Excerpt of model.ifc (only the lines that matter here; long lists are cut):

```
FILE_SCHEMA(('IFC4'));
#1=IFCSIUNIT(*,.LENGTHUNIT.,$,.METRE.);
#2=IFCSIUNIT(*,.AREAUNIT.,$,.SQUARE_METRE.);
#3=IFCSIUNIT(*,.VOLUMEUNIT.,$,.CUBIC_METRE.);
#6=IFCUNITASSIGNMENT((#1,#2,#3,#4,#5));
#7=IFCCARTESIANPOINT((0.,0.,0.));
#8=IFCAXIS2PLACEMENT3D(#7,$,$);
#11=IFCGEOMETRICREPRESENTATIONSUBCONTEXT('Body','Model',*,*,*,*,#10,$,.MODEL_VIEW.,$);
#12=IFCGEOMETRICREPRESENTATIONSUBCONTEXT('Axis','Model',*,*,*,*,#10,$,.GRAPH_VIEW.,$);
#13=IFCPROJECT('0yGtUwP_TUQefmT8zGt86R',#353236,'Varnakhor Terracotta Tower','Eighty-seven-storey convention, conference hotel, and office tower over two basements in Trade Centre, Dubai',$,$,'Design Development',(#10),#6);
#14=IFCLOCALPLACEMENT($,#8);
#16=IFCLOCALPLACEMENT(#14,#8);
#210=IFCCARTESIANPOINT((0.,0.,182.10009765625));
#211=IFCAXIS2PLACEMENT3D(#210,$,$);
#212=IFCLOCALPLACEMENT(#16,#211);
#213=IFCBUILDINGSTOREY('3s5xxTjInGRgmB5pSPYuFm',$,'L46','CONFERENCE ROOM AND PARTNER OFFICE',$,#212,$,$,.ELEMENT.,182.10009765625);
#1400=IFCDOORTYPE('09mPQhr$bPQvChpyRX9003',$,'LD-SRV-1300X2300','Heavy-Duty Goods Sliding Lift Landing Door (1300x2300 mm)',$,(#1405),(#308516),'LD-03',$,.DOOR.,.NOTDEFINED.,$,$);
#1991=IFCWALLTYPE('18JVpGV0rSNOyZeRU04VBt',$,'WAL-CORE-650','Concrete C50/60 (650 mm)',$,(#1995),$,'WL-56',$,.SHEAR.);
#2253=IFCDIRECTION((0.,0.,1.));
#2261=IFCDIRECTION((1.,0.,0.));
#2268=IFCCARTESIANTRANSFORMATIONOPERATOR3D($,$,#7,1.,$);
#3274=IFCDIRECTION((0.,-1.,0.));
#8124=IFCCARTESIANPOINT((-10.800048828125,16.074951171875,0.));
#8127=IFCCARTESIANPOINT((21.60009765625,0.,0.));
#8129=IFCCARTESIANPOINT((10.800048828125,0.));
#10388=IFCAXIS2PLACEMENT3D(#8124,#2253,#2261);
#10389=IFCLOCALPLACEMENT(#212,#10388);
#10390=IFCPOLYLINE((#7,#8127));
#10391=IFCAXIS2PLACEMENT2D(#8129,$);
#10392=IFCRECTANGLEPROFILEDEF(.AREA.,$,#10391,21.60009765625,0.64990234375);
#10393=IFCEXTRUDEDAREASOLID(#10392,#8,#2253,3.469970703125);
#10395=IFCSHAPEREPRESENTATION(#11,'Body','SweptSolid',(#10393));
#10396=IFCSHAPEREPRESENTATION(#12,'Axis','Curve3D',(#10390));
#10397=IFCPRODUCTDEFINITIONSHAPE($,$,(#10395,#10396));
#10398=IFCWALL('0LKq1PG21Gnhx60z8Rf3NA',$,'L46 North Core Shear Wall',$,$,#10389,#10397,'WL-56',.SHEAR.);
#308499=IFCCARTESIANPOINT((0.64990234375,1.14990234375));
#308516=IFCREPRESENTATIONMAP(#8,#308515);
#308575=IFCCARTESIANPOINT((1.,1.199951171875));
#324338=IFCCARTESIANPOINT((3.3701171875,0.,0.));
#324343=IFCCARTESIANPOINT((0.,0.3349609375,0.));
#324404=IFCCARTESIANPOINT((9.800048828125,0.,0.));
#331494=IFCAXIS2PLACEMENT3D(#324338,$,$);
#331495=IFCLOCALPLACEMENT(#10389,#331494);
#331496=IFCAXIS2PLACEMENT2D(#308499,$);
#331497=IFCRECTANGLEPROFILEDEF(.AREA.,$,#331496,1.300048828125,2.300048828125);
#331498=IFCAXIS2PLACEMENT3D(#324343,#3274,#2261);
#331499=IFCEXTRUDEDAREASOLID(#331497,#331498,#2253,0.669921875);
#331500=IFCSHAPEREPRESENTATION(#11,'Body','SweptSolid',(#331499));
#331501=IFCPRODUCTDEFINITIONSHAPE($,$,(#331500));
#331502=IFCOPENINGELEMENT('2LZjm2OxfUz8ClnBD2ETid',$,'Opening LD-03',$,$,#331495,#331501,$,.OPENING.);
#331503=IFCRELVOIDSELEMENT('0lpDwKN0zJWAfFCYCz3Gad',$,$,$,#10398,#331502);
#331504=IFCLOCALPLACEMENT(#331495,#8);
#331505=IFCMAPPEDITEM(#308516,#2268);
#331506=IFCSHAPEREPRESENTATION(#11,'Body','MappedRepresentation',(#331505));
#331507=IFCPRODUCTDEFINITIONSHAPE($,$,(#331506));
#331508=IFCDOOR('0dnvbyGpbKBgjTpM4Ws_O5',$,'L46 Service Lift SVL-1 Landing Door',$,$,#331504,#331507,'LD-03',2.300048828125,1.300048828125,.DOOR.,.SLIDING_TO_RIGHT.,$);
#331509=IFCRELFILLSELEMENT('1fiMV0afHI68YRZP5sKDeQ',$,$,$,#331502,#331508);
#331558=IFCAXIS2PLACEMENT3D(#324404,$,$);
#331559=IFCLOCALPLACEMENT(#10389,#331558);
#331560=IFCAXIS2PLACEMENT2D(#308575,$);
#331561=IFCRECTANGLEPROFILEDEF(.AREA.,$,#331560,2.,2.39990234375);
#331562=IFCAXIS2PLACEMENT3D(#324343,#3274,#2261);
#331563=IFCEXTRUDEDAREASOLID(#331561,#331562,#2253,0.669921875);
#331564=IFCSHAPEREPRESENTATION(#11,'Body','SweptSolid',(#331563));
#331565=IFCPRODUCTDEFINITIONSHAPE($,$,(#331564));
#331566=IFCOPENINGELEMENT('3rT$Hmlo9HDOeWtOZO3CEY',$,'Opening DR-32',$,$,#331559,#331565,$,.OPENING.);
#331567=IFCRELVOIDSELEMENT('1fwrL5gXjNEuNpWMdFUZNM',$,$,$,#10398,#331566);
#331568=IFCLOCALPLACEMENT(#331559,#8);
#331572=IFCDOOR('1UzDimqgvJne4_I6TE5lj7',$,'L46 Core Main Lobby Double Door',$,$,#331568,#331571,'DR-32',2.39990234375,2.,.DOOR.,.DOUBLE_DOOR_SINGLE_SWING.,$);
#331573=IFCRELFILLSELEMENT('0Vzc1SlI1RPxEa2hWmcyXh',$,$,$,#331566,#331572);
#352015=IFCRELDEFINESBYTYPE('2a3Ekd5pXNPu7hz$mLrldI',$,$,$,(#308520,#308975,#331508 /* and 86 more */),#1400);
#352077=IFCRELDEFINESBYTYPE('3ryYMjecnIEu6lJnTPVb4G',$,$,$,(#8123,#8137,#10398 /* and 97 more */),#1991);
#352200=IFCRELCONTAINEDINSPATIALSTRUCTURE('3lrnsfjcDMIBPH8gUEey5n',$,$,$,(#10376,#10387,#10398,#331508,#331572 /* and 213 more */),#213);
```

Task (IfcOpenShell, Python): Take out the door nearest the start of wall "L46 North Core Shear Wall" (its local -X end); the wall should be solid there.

```python
import ifcopenshell
import ifcopenshell.api.feature
import ifcopenshell.api.root
import ifcopenshell.geom
import ifcopenshell.util.shape

model = ifcopenshell.open("model.ifc")
settings = ifcopenshell.geom.settings()


def volume(element):
    """Net volume in cubic metres, openings subtracted."""
    shape = ifcopenshell.geom.create_shape(settings, element)
    return ifcopenshell.util.shape.get_volume(shape.geometry)


door = model.by_guid("0dnvbyGpbKBgjTpM4Ws_O5")
opening = door.FillsVoids[0].RelatingOpeningElement
wall = opening.VoidsElements[0].RelatingBuildingElement
before = volume(wall)

ifcopenshell.api.root.remove_product(model, product=door)
ifcopenshell.api.feature.remove_feature(model, feature=opening)

after = volume(wall)

print(f"wall volume {before:.3f} -> {after:.3f} m3")

model.write("model_v2.ifc")
```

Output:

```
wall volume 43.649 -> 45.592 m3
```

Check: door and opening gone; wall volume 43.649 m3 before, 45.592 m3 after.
